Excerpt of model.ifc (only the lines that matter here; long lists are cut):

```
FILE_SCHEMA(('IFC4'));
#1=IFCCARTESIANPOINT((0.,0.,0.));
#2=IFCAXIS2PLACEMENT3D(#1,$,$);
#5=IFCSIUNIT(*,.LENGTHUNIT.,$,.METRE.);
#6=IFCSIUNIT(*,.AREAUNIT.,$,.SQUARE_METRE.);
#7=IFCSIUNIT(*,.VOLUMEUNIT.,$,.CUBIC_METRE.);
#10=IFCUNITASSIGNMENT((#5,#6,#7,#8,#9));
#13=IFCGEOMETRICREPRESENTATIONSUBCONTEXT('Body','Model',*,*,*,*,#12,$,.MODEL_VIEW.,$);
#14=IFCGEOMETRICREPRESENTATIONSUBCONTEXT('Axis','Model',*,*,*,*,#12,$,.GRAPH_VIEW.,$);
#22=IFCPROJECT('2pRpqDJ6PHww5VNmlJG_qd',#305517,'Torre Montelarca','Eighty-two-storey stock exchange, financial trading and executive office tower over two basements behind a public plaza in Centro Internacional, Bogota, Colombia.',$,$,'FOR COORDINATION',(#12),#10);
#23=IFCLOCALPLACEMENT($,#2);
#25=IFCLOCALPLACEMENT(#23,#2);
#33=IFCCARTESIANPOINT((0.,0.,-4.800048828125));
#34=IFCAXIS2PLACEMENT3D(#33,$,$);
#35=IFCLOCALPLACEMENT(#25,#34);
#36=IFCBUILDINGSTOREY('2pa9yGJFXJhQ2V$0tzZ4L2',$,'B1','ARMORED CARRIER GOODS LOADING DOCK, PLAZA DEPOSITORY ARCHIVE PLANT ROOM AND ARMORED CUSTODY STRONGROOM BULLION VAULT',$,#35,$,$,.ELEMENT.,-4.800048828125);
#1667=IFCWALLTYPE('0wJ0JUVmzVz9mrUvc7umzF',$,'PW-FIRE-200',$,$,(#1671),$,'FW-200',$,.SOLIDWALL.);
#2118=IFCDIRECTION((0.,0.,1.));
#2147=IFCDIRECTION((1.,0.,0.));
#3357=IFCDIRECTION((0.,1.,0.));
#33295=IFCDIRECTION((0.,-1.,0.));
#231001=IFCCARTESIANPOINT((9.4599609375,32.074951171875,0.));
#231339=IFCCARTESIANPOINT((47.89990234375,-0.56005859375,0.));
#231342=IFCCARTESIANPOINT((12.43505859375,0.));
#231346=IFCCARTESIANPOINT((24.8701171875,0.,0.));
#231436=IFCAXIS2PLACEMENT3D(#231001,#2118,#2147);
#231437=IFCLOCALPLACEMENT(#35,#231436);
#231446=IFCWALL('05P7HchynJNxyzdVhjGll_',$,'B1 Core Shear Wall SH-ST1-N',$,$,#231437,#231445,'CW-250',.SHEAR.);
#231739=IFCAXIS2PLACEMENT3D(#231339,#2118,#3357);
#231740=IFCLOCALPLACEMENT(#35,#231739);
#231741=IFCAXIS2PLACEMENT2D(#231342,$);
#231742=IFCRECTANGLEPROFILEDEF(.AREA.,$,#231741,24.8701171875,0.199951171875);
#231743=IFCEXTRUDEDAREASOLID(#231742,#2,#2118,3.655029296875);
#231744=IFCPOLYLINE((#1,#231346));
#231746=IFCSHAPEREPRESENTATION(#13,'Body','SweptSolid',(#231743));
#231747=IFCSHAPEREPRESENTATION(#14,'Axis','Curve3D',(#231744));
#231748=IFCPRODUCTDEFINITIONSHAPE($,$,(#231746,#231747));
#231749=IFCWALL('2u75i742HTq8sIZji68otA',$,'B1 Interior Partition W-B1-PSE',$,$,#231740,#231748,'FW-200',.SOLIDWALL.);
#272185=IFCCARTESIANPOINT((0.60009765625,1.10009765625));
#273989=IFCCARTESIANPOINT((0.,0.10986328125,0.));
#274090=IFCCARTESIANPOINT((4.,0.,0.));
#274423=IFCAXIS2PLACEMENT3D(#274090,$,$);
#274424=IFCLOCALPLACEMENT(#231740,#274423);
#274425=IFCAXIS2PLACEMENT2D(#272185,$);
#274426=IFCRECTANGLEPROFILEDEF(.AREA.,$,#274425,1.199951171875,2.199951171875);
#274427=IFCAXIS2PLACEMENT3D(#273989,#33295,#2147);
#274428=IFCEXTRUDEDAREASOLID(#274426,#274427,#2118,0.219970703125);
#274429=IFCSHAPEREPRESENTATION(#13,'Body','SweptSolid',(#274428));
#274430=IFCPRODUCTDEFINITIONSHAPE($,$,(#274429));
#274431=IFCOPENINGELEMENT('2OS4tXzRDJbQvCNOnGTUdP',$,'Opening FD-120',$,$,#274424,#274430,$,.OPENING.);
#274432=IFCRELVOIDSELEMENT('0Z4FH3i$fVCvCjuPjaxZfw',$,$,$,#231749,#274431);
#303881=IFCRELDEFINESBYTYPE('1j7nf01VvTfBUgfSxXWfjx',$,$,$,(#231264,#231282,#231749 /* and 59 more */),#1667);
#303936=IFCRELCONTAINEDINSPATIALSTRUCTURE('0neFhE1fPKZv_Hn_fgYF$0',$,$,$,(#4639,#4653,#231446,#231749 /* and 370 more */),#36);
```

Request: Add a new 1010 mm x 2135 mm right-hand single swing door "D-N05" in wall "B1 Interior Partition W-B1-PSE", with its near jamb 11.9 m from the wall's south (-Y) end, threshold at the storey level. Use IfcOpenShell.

```python
import numpy as np
import ifcopenshell
import ifcopenshell.api.feature
import ifcopenshell.api.geometry
import ifcopenshell.api.root
import ifcopenshell.api.spatial
import ifcopenshell.geom
import ifcopenshell.util.element
import ifcopenshell.util.placement
import ifcopenshell.util.representation
import ifcopenshell.util.shape
import ifcopenshell.util.unit

model = ifcopenshell.open("model.ifc")
unit_scale = ifcopenshell.util.unit.calculate_unit_scale(model)
settings = ifcopenshell.geom.settings()


def volume(element):
    """Net volume in cubic metres, openings subtracted."""
    shape = ifcopenshell.geom.create_shape(settings, element)
    return ifcopenshell.util.shape.get_volume(shape.geometry)


wall = model.by_id(231749)
storey = ifcopenshell.util.element.get_container(wall, ifc_class="IfcBuildingStorey")
context = ifcopenshell.util.representation.get_context(model, "Model", "Body", "MODEL_VIEW")
before = volume(wall)

width, height, from_end, sill = 1.01, 2.135, 11.9, 0.0  # metres

# The wall runs along its own X axis, and the end named is its -X end.
wall_shape = ifcopenshell.geom.create_shape(settings, wall)
x, y, z = ifcopenshell.util.shape.get_vertices(wall_shape.geometry).T
start = x.min() + from_end
face, thickness = float(y.min()), float(y.max() - y.min())
wall_matrix = ifcopenshell.util.placement.get_local_placement(wall.ObjectPlacement)
level = ifcopenshell.util.placement.get_local_placement(storey.ObjectPlacement)[2, 3]


def in_wall(x, y):
    """Placement at x, y metres in the wall's axes, at sill height."""
    matrix = wall_matrix.copy()
    matrix[:, 3] = wall_matrix @ np.array([x / unit_scale, y / unit_scale, 0.0, 1.0])
    matrix[2, 3] = level + sill / unit_scale
    return matrix


# Opening: a box that overshoots both wall faces by 50 mm.
opening = ifcopenshell.api.root.create_entity(model, ifc_class="IfcOpeningElement", predefined_type="OPENING")
box = ifcopenshell.api.geometry.add_wall_representation(
    model, context=context, length=width, height=height, thickness=thickness + 0.1
)
ifcopenshell.api.geometry.assign_representation(model, product=opening, representation=box)
ifcopenshell.api.geometry.edit_object_placement(model, product=opening, matrix=in_wall(start, face - 0.05), is_si=False)
ifcopenshell.api.feature.add_feature(model, feature=opening, element=wall)

door = ifcopenshell.api.root.create_entity(model, ifc_class="IfcDoor", name="D-N05", predefined_type="DOOR")
door.OverallWidth, door.OverallHeight = width / unit_scale, height / unit_scale
door.OperationType = "SINGLE_SWING_RIGHT"
body = ifcopenshell.api.geometry.add_door_representation(
    model,
    context=context,
    overall_width=door.OverallWidth,
    overall_height=door.OverallHeight,
    operation_type="SINGLE_SWING_RIGHT",
    lining_properties={"LiningDepth": thickness / unit_scale, "ThresholdDepth": thickness / unit_scale},
)
ifcopenshell.api.geometry.assign_representation(model, product=door, representation=body)
ifcopenshell.api.spatial.assign_container(model, products=[door], relating_structure=storey)
ifcopenshell.api.feature.add_filling(model, opening=opening, element=door)

# The lining spans the wall, so the door starts at the wall face.
ifcopenshell.api.geometry.edit_object_placement(model, product=door, matrix=in_wall(start, face), is_si=False)

after = volume(wall)

print(f"wall volume {before:.3f} -> {after:.3f} m3")

model.write("model_updated.ifc")
```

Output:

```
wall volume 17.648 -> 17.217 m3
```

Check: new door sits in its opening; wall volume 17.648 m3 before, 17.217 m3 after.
